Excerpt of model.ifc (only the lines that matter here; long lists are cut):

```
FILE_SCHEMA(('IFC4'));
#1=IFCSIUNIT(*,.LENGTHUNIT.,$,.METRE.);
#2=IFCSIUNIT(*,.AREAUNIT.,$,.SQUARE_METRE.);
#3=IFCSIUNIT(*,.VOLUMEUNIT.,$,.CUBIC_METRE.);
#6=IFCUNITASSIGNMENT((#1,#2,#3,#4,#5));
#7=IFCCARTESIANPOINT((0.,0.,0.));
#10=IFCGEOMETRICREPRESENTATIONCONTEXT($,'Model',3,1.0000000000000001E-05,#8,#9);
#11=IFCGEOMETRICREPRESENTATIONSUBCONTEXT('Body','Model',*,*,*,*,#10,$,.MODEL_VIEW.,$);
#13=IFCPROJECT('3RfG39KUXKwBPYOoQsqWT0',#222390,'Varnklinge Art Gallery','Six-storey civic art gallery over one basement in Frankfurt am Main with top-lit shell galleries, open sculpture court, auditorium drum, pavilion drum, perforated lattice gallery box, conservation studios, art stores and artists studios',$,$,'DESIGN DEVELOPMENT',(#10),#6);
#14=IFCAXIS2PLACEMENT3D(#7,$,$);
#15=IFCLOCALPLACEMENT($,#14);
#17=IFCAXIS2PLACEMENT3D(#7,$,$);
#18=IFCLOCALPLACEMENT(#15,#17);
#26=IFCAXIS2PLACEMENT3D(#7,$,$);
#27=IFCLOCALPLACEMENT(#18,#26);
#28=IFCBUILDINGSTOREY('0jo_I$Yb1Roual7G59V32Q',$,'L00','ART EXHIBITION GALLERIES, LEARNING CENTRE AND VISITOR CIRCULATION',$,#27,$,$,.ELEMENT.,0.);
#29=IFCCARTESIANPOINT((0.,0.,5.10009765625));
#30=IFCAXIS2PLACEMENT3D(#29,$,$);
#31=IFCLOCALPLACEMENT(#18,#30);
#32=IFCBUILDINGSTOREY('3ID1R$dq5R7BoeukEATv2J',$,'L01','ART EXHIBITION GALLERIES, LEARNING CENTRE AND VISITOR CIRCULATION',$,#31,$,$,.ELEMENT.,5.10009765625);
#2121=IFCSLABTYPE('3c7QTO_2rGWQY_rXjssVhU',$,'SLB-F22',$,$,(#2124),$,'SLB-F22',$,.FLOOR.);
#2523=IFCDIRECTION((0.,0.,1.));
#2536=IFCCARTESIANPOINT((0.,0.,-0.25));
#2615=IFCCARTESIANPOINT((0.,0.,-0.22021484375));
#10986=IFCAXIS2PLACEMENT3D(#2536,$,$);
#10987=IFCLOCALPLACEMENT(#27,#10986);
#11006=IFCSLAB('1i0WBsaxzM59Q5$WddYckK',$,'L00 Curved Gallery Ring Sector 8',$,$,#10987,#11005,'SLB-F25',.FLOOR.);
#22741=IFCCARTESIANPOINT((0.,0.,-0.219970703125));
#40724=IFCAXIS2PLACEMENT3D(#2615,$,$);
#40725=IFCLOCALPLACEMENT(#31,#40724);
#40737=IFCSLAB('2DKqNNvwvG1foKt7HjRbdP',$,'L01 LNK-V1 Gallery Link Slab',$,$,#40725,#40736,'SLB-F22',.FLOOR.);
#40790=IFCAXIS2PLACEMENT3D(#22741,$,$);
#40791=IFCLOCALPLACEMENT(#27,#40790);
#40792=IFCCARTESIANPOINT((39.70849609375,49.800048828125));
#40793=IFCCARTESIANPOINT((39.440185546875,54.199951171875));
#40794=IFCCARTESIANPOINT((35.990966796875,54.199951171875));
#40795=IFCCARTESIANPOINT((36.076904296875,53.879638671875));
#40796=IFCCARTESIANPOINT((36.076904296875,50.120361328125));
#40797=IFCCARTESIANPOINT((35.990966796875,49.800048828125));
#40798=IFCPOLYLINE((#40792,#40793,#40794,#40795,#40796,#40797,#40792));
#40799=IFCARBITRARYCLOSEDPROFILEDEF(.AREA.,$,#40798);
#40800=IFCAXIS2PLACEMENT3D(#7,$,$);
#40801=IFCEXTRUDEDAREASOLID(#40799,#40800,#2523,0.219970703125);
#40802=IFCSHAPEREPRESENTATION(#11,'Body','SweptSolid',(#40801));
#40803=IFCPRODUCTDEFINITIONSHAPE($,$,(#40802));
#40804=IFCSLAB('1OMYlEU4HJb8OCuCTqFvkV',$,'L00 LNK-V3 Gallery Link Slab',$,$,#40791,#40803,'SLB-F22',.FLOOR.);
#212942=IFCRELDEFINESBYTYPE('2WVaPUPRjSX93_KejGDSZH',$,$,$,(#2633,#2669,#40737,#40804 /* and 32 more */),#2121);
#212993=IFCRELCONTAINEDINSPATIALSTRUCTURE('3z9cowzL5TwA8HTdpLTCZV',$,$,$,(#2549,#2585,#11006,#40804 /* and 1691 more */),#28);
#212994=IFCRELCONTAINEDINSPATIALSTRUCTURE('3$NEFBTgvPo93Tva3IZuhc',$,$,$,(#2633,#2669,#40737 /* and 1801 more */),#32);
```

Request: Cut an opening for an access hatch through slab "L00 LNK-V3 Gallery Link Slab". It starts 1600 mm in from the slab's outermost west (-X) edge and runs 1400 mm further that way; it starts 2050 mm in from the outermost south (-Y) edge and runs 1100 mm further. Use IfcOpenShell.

```python
import numpy as np
import ifcopenshell
import ifcopenshell.api.feature
import ifcopenshell.api.geometry
import ifcopenshell.api.root
import ifcopenshell.geom
import ifcopenshell.util.placement
import ifcopenshell.util.representation
import ifcopenshell.util.shape
import ifcopenshell.util.unit

model = ifcopenshell.open("model.ifc")
unit_scale = ifcopenshell.util.unit.calculate_unit_scale(model)
settings = ifcopenshell.geom.settings()


def volume(element):
    """Net volume in cubic metres, openings subtracted."""
    shape = ifcopenshell.geom.create_shape(settings, element)
    return ifcopenshell.util.shape.get_volume(shape.geometry)


slab = model.by_guid("1OMYlEU4HJb8OCuCTqFvkV")
before = volume(slab)

# Extent in the slab's own axes, in metres. The edges named are its -X and -Y sides.
slab_shape = ifcopenshell.geom.create_shape(settings, slab)
vertices = ifcopenshell.util.shape.get_vertices(slab_shape.geometry)
x_min, y_min, bottom = vertices.min(axis=0)
top = vertices[:, 2].max()

opening = ifcopenshell.api.root.create_entity(model, ifc_class="IfcOpeningElement", name="Access hatch opening", predefined_type="OPENING")
context = ifcopenshell.util.representation.get_context(model, "Model", "Body", "MODEL_VIEW")
width, depth = 1.4, 1.1
outline = [(0.0, 0.0), (width, 0.0), (width, depth), (0.0, depth), (0.0, 0.0)]
# Overshoot both faces by 50 mm so the cut is clean.
shape = ifcopenshell.api.geometry.add_slab_representation(
    model, context=context, depth=top - bottom + 0.1, polyline=outline
)
ifcopenshell.api.geometry.assign_representation(model, product=opening, representation=shape)

matrix = ifcopenshell.util.placement.get_local_placement(slab.ObjectPlacement)
matrix[:, 3] = matrix @ np.append(np.array([x_min + 1.6, y_min + 2.05, bottom - 0.05]) / unit_scale, 1.0)
ifcopenshell.api.geometry.edit_object_placement(model, product=opening, matrix=matrix, is_si=False)
ifcopenshell.api.feature.add_feature(model, feature=opening, element=slab)

after = volume(slab)

print(f"slab volume {before:.3f} -> {after:.3f} m3")

model.write("model_v2.ifc")
```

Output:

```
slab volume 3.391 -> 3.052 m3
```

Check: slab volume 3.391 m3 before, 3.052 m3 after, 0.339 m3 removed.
